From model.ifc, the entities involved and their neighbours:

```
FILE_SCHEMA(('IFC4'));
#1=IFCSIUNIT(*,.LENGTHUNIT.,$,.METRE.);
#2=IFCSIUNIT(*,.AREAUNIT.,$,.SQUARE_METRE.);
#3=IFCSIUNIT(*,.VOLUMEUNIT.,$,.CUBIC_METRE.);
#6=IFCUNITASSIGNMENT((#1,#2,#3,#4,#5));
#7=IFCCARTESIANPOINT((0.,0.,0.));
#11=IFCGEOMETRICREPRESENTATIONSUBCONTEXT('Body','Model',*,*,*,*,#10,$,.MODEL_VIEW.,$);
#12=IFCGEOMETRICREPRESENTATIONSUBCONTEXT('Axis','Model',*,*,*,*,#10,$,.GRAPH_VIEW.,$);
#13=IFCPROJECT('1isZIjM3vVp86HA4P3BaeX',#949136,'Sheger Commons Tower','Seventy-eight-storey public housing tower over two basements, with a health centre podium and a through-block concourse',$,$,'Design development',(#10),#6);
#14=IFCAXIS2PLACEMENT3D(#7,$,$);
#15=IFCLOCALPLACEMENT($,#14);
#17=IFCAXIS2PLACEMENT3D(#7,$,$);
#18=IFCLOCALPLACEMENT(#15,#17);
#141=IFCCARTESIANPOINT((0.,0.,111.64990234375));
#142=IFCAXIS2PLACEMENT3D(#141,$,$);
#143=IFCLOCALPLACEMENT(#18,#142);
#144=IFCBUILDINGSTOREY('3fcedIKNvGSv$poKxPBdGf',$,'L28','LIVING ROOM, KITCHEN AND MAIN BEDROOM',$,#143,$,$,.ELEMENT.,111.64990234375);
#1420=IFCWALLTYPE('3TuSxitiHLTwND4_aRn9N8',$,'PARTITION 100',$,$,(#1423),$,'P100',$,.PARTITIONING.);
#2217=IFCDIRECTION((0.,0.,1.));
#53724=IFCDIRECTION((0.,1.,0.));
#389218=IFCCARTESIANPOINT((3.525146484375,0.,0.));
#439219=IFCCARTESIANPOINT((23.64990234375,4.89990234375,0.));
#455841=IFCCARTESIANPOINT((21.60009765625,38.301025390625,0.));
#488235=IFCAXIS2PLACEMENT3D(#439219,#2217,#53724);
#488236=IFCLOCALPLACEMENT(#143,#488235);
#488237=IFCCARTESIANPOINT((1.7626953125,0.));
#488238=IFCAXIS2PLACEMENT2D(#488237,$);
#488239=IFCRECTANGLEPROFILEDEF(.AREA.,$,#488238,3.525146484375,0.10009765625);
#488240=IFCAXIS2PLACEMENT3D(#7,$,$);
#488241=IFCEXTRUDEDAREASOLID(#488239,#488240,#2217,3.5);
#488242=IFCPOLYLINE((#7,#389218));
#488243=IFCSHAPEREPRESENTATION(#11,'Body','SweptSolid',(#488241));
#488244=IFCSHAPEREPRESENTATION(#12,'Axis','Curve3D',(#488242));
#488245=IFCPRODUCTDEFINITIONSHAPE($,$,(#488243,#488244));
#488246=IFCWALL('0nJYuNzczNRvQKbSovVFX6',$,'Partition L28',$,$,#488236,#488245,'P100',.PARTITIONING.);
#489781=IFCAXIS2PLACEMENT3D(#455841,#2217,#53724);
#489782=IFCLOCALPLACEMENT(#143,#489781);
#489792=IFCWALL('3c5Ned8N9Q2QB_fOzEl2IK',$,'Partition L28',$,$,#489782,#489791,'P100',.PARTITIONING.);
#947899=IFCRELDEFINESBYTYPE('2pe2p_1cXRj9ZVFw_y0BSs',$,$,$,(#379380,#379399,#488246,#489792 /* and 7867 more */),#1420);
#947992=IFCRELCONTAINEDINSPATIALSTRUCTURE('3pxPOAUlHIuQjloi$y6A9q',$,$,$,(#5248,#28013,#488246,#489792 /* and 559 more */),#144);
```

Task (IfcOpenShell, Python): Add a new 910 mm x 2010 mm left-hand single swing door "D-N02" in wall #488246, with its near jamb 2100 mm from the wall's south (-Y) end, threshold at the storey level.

```python
import numpy as np
import ifcopenshell
import ifcopenshell.api.feature
import ifcopenshell.api.geometry
import ifcopenshell.api.root
import ifcopenshell.api.spatial
import ifcopenshell.geom
import ifcopenshell.util.element
import ifcopenshell.util.placement
import ifcopenshell.util.representation
import ifcopenshell.util.shape
import ifcopenshell.util.unit

model = ifcopenshell.open("model.ifc")
unit_scale = ifcopenshell.util.unit.calculate_unit_scale(model)
settings = ifcopenshell.geom.settings()


def volume(element):
    """Net volume in cubic metres, openings subtracted."""
    shape = ifcopenshell.geom.create_shape(settings, element)
    return ifcopenshell.util.shape.get_volume(shape.geometry)


wall = model.by_guid("0nJYuNzczNRvQKbSovVFX6")
storey = ifcopenshell.util.element.get_container(wall, ifc_class="IfcBuildingStorey")
context = ifcopenshell.util.representation.get_context(model, "Model", "Body", "MODEL_VIEW")
before = volume(wall)

width, height, from_end, sill = 0.91, 2.01, 2.1, 0.0  # metres

# The wall runs along its own X axis, and the end named is its -X end.
wall_shape = ifcopenshell.geom.create_shape(settings, wall)
x, y, z = ifcopenshell.util.shape.get_vertices(wall_shape.geometry).T
start = x.min() + from_end
face, thickness = float(y.min()), float(y.max() - y.min())
wall_matrix = ifcopenshell.util.placement.get_local_placement(wall.ObjectPlacement)
level = ifcopenshell.util.placement.get_local_placement(storey.ObjectPlacement)[2, 3]


def in_wall(x, y):
    """Placement at x, y metres in the wall's axes, at sill height."""
    matrix = wall_matrix.copy()
    matrix[:, 3] = wall_matrix @ np.array([x / unit_scale, y / unit_scale, 0.0, 1.0])
    matrix[2, 3] = level + sill / unit_scale
    return matrix


# Opening: a box that overshoots both wall faces by 50 mm.
opening = ifcopenshell.api.root.create_entity(model, ifc_class="IfcOpeningElement", predefined_type="OPENING")
box = ifcopenshell.api.geometry.add_wall_representation(
    model, context=context, length=width, height=height, thickness=thickness + 0.1
)
ifcopenshell.api.geometry.assign_representation(model, product=opening, representation=box)
ifcopenshell.api.geometry.edit_object_placement(model, product=opening, matrix=in_wall(start, face - 0.05), is_si=False)
ifcopenshell.api.feature.add_feature(model, feature=opening, element=wall)

door = ifcopenshell.api.root.create_entity(model, ifc_class="IfcDoor", name="D-N02", predefined_type="DOOR")
door.OverallWidth, door.OverallHeight = width / unit_scale, height / unit_scale
door.OperationType = "SINGLE_SWING_LEFT"
body = ifcopenshell.api.geometry.add_door_representation(
    model,
    context=context,
    overall_width=door.OverallWidth,
    overall_height=door.OverallHeight,
    operation_type="SINGLE_SWING_LEFT",
    lining_properties={"LiningDepth": thickness / unit_scale, "ThresholdDepth": thickness / unit_scale},
)
ifcopenshell.api.geometry.assign_representation(model, product=door, representation=body)
ifcopenshell.api.spatial.assign_container(model, products=[door], relating_structure=storey)
ifcopenshell.api.feature.add_filling(model, opening=opening, element=door)

# The lining spans the wall, so the door starts at the wall face.
ifcopenshell.api.geometry.edit_object_placement(model, product=door, matrix=in_wall(start, face), is_si=False)

after = volume(wall)

print(f"wall volume {before:.3f} -> {after:.3f} m3")

model.write("model_updated.ifc")
```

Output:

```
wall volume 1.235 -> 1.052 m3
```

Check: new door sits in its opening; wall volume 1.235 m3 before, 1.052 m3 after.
